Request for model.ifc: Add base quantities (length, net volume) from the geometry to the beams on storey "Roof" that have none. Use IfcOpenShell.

First a look at what the model holds.

```python
import ifcopenshell
import ifcopenshell.util.element
import ifcopenshell.util.unit

model = ifcopenshell.open("model.ifc")
print(model.schema)
for unit_type in ("LENGTHUNIT", "AREAUNIT", "VOLUMEUNIT"):
    print(unit_type, ifcopenshell.util.unit.calculate_unit_scale(model, unit_type))
storey = next(s for s in model.by_type("IfcBuildingStorey") if s.Name == "Roof")
beams = [e for e in ifcopenshell.util.element.get_decomposition(storey) if e.is_a("IfcBeam")]
for e in sorted(beams, key=lambda e: e.id()):
    print(e.id(), e.is_a(), e.Name, list(ifcopenshell.util.element.get_psets(e, qtos_only=True)), sep=" | ")
```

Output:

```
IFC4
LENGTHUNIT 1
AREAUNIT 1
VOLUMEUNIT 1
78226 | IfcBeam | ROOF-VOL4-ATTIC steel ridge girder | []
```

```python
import ifcopenshell
import ifcopenshell.api.pset
import ifcopenshell.geom
import ifcopenshell.util.element
import ifcopenshell.util.shape
import ifcopenshell.util.unit

model = ifcopenshell.open("model.ifc")
unit_scale = ifcopenshell.util.unit.calculate_unit_scale(model)
volume_scale = ifcopenshell.util.unit.calculate_unit_scale(model, "VOLUMEUNIT")
settings = ifcopenshell.geom.settings()

storey = next(s for s in model.by_type("IfcBuildingStorey") if s.Name == "Roof")
beams = [e for e in ifcopenshell.util.element.get_decomposition(storey) if e.is_a("IfcBeam")]

for e in sorted(beams, key=lambda e: e.id()):
    if ifcopenshell.util.element.get_psets(e, qtos_only=True, should_inherit=False):
        continue
    # Geometry comes back in metres, in the element's own axes.
    shape = ifcopenshell.geom.create_shape(settings, e)
    values = {
        "Length": ifcopenshell.util.shape.get_max_xyz(shape.geometry) / unit_scale,
        "NetVolume": ifcopenshell.util.shape.get_volume(shape.geometry) / volume_scale,
    }
    qto = ifcopenshell.api.pset.add_qto(model, product=e, name="Qto_BeamBaseQuantities")
    ifcopenshell.api.pset.edit_qto(model, qto=qto, properties=values)
    print(e.id(), {k: round(v, 3) for k, v in values.items()})

model.write("model_edited.ifc")
```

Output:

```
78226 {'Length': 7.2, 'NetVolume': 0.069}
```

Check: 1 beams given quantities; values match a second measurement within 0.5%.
